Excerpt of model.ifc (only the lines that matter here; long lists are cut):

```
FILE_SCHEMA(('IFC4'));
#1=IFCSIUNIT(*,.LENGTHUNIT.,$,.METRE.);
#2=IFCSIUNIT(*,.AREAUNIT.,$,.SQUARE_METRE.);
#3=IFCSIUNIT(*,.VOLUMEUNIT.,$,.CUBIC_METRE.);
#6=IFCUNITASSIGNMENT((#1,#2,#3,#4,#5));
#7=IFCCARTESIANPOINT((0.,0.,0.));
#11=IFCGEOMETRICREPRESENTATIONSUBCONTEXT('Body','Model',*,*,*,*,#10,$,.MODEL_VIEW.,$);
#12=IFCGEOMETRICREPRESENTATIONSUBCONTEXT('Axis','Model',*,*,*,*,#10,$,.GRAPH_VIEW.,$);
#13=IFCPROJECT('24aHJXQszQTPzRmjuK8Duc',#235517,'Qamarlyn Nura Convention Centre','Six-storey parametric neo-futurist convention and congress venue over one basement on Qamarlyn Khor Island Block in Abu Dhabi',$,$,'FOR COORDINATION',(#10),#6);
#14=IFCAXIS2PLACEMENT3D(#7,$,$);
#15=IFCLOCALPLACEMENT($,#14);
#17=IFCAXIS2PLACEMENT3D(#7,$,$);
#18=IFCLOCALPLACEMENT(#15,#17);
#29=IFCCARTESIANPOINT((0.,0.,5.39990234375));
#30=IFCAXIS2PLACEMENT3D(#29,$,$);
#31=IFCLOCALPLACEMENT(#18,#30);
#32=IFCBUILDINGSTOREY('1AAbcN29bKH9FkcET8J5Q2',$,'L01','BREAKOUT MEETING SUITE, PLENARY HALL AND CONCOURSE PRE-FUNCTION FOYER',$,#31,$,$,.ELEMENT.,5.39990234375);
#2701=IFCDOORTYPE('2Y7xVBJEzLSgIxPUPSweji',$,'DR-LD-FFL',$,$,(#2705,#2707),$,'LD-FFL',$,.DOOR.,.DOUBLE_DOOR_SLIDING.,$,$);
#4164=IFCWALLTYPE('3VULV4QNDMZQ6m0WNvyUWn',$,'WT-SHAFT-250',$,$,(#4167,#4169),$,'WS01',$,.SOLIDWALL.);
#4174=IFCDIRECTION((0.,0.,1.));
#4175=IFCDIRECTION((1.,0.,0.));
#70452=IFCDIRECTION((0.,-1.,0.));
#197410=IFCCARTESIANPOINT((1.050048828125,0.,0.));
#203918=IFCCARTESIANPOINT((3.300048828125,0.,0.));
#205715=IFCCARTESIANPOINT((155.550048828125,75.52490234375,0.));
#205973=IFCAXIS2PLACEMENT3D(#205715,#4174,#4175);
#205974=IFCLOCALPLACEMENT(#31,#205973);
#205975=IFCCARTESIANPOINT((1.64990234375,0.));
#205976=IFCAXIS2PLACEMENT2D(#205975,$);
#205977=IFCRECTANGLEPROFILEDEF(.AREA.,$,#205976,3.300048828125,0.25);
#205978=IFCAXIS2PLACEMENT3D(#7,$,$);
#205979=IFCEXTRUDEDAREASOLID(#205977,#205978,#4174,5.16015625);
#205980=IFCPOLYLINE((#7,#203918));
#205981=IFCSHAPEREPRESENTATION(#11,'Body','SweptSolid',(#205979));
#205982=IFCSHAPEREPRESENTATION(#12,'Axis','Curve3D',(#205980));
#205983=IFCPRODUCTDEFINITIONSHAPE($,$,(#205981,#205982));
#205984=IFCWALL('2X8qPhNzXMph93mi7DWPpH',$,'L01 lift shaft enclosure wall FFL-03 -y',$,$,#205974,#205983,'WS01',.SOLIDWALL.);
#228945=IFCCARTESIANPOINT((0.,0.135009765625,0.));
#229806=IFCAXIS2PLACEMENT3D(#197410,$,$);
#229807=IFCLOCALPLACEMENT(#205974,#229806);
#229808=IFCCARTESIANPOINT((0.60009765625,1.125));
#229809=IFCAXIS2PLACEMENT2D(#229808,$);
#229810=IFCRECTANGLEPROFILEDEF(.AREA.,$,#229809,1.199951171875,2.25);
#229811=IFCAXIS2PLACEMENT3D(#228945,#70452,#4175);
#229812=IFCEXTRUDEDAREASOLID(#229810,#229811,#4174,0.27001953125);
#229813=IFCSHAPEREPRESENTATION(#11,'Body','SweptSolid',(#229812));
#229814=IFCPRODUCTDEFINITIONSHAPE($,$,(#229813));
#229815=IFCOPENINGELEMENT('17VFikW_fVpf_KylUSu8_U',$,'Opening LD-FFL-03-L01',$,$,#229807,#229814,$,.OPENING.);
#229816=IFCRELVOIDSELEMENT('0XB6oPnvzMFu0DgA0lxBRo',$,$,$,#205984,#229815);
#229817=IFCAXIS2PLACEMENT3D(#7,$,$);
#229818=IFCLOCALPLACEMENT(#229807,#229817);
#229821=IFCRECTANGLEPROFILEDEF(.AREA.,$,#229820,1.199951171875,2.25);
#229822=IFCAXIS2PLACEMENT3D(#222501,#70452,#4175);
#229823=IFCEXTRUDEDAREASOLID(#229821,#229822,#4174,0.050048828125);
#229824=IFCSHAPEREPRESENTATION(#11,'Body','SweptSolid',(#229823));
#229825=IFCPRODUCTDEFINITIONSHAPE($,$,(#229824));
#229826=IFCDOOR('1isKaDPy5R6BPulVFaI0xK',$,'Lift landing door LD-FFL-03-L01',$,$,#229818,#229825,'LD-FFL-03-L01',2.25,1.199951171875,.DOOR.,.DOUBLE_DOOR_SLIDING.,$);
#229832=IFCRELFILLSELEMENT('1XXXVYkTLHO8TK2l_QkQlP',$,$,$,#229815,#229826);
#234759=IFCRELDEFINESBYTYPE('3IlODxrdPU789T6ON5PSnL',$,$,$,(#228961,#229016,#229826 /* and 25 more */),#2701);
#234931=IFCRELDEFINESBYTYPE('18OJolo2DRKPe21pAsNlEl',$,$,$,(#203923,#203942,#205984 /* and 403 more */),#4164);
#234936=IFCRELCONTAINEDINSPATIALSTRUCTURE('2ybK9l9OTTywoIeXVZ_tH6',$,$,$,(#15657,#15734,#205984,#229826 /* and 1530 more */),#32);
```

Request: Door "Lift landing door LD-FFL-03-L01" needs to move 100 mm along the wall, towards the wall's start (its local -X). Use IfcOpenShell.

```python
import ifcopenshell
import ifcopenshell.api.geometry
import ifcopenshell.util.placement
import ifcopenshell.util.unit

model = ifcopenshell.open("model.ifc")
unit_scale = ifcopenshell.util.unit.calculate_unit_scale(model)

door = model.by_id(229826)
opening = door.FillsVoids[0].RelatingOpeningElement
wall = opening.VoidsElements[0].RelatingBuildingElement

wall_matrix = ifcopenshell.util.placement.get_local_placement(wall.ObjectPlacement)
shift = wall_matrix[:3, 0] * -0.1 / unit_scale
before = ifcopenshell.util.placement.get_local_placement(door.ObjectPlacement)[:3, 3].copy()

# The door is placed relative to its opening, so it follows when the opening moves.
matrix = ifcopenshell.util.placement.get_local_placement(opening.ObjectPlacement)
matrix[:3, 3] += shift
ifcopenshell.api.geometry.edit_object_placement(
    model, product=opening, matrix=matrix, is_si=False, should_transform_children=True
)

after = ifcopenshell.util.placement.get_local_placement(door.ObjectPlacement)[:3, 3]
print("door moved by", (after - before).round(3) + 0.0)

model.write("model_updated.ifc")
```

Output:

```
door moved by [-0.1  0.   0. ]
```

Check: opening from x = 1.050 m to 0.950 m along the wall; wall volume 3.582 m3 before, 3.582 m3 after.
